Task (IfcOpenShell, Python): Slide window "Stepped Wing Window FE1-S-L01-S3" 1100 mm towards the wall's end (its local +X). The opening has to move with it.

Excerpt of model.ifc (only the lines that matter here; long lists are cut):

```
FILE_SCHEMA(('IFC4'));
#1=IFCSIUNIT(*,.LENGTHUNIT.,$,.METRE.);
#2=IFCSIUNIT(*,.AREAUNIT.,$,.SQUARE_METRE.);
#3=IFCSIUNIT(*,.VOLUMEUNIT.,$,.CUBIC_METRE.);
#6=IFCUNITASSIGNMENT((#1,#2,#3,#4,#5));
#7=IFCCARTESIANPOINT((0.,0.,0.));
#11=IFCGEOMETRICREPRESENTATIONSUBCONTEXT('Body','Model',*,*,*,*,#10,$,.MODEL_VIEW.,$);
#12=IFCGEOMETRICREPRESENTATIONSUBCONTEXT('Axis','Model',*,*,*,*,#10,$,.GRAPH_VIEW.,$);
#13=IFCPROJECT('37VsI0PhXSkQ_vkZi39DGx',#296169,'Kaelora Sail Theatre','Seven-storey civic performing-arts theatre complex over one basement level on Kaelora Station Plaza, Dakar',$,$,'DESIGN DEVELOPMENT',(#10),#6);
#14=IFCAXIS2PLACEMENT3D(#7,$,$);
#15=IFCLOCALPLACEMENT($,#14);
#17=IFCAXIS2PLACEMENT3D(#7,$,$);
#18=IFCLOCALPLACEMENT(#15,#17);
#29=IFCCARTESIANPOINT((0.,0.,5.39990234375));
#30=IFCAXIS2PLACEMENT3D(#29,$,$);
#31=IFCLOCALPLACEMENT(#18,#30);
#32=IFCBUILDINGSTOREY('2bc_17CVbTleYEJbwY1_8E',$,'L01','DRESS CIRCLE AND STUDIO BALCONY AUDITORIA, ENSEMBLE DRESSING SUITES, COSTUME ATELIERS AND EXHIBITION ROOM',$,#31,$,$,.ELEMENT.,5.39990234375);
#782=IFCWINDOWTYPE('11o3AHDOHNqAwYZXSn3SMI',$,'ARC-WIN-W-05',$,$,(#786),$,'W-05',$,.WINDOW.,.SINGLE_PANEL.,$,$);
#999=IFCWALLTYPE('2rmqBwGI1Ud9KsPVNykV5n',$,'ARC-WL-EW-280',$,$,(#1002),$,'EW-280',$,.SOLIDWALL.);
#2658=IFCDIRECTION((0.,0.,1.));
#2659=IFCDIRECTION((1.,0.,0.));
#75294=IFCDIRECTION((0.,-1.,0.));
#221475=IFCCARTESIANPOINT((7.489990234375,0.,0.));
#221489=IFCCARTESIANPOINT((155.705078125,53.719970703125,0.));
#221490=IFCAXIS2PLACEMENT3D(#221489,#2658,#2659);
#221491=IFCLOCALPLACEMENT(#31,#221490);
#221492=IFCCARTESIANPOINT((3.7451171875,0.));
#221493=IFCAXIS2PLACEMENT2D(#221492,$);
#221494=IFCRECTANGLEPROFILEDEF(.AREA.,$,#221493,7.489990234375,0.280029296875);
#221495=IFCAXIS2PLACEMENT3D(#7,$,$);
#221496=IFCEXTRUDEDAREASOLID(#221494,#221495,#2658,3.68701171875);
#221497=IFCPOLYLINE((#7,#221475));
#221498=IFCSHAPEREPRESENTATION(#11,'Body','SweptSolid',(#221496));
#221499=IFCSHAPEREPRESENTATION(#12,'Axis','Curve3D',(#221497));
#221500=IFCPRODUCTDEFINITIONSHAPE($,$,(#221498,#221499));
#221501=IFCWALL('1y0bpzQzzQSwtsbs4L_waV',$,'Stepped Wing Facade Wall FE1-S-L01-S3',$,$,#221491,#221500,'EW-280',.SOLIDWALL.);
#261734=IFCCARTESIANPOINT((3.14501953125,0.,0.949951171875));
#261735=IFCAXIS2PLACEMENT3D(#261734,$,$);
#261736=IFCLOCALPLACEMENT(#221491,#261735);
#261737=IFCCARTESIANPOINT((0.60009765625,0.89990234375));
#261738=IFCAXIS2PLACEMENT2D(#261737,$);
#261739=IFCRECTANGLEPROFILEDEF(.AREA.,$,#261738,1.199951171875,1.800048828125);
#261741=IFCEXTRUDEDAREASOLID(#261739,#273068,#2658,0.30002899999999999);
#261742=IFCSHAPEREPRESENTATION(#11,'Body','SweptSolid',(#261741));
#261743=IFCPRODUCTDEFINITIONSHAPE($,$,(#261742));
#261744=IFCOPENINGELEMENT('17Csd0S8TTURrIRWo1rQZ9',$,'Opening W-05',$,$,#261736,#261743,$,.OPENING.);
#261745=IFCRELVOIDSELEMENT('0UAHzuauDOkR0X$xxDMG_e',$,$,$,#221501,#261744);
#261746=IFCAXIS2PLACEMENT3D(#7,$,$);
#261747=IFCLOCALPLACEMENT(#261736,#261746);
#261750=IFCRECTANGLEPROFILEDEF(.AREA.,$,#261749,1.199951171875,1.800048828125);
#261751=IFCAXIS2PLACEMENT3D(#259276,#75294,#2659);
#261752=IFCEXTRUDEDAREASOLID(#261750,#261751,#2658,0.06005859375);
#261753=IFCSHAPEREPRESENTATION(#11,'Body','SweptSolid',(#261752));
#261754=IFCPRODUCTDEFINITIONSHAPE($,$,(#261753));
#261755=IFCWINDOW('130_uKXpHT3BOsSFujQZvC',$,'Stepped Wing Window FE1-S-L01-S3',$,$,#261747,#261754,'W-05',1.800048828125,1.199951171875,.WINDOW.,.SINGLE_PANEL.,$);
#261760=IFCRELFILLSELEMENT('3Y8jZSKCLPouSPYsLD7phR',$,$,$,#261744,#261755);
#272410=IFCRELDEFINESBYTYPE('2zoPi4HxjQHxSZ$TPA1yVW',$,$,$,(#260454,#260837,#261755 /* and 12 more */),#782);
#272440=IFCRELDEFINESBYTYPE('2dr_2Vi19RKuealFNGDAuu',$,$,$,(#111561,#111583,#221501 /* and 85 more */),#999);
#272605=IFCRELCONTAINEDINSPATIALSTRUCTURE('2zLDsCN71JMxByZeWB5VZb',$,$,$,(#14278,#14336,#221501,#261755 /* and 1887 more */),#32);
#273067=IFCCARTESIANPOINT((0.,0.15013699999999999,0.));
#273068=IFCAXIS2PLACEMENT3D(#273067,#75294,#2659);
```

```python
import ifcopenshell
import ifcopenshell.api.geometry
import ifcopenshell.util.placement
import ifcopenshell.util.unit

model = ifcopenshell.open("model.ifc")
unit_scale = ifcopenshell.util.unit.calculate_unit_scale(model)

window = model.by_id(261755)
opening = window.FillsVoids[0].RelatingOpeningElement
wall = opening.VoidsElements[0].RelatingBuildingElement

wall_matrix = ifcopenshell.util.placement.get_local_placement(wall.ObjectPlacement)
shift = wall_matrix[:3, 0] * 1.1 / unit_scale
before = ifcopenshell.util.placement.get_local_placement(window.ObjectPlacement)[:3, 3].copy()

# The window is placed relative to its opening, so it follows when the opening moves.
matrix = ifcopenshell.util.placement.get_local_placement(opening.ObjectPlacement)
matrix[:3, 3] += shift
ifcopenshell.api.geometry.edit_object_placement(
    model, product=opening, matrix=matrix, is_si=False, should_transform_children=True
)

after = ifcopenshell.util.placement.get_local_placement(window.ObjectPlacement)[:3, 3]
print("window moved by", (after - before).round(3) + 0.0)

model.write("model_edited.ifc")
```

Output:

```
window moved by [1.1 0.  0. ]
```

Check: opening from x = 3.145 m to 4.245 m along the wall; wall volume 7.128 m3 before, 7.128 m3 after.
